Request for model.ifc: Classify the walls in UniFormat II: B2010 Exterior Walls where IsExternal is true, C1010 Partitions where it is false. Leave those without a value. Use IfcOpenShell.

First a look at what the model holds.

```python
import ifcopenshell
import ifcopenshell.util.element

model = ifcopenshell.open("model.ifc")
print(model.schema)
print("classifications:", [c.Name for c in model.by_type("IfcClassification")])
values = [ifcopenshell.util.element.get_pset(e, "Pset_WallCommon", "IsExternal") for e in model.by_type("IfcWall")]
for value in (True, False, None):
    print("IsExternal", value, values.count(value))
```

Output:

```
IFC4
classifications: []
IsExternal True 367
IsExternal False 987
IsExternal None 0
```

```python
import ifcopenshell
import ifcopenshell.api.classification
import ifcopenshell.util.element

model = ifcopenshell.open("model.ifc")

system = ifcopenshell.api.classification.add_classification(model, classification="UniFormat II")

walls = model.by_type("IfcWall")
external = {e: ifcopenshell.util.element.get_pset(e, "Pset_WallCommon", "IsExternal") for e in walls}
for flag, code, name in ((True, "B2010", "Exterior Walls"), (False, "C1010", "Partitions")):
    products = [e for e in walls if external[e] is flag]
    ifcopenshell.api.classification.add_reference(
        model, products=products, classification=system, identification=code, name=name
    )
    print(code, len(products))

model.write("model_v2.ifc")
```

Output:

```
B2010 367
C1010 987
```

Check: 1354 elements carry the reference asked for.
